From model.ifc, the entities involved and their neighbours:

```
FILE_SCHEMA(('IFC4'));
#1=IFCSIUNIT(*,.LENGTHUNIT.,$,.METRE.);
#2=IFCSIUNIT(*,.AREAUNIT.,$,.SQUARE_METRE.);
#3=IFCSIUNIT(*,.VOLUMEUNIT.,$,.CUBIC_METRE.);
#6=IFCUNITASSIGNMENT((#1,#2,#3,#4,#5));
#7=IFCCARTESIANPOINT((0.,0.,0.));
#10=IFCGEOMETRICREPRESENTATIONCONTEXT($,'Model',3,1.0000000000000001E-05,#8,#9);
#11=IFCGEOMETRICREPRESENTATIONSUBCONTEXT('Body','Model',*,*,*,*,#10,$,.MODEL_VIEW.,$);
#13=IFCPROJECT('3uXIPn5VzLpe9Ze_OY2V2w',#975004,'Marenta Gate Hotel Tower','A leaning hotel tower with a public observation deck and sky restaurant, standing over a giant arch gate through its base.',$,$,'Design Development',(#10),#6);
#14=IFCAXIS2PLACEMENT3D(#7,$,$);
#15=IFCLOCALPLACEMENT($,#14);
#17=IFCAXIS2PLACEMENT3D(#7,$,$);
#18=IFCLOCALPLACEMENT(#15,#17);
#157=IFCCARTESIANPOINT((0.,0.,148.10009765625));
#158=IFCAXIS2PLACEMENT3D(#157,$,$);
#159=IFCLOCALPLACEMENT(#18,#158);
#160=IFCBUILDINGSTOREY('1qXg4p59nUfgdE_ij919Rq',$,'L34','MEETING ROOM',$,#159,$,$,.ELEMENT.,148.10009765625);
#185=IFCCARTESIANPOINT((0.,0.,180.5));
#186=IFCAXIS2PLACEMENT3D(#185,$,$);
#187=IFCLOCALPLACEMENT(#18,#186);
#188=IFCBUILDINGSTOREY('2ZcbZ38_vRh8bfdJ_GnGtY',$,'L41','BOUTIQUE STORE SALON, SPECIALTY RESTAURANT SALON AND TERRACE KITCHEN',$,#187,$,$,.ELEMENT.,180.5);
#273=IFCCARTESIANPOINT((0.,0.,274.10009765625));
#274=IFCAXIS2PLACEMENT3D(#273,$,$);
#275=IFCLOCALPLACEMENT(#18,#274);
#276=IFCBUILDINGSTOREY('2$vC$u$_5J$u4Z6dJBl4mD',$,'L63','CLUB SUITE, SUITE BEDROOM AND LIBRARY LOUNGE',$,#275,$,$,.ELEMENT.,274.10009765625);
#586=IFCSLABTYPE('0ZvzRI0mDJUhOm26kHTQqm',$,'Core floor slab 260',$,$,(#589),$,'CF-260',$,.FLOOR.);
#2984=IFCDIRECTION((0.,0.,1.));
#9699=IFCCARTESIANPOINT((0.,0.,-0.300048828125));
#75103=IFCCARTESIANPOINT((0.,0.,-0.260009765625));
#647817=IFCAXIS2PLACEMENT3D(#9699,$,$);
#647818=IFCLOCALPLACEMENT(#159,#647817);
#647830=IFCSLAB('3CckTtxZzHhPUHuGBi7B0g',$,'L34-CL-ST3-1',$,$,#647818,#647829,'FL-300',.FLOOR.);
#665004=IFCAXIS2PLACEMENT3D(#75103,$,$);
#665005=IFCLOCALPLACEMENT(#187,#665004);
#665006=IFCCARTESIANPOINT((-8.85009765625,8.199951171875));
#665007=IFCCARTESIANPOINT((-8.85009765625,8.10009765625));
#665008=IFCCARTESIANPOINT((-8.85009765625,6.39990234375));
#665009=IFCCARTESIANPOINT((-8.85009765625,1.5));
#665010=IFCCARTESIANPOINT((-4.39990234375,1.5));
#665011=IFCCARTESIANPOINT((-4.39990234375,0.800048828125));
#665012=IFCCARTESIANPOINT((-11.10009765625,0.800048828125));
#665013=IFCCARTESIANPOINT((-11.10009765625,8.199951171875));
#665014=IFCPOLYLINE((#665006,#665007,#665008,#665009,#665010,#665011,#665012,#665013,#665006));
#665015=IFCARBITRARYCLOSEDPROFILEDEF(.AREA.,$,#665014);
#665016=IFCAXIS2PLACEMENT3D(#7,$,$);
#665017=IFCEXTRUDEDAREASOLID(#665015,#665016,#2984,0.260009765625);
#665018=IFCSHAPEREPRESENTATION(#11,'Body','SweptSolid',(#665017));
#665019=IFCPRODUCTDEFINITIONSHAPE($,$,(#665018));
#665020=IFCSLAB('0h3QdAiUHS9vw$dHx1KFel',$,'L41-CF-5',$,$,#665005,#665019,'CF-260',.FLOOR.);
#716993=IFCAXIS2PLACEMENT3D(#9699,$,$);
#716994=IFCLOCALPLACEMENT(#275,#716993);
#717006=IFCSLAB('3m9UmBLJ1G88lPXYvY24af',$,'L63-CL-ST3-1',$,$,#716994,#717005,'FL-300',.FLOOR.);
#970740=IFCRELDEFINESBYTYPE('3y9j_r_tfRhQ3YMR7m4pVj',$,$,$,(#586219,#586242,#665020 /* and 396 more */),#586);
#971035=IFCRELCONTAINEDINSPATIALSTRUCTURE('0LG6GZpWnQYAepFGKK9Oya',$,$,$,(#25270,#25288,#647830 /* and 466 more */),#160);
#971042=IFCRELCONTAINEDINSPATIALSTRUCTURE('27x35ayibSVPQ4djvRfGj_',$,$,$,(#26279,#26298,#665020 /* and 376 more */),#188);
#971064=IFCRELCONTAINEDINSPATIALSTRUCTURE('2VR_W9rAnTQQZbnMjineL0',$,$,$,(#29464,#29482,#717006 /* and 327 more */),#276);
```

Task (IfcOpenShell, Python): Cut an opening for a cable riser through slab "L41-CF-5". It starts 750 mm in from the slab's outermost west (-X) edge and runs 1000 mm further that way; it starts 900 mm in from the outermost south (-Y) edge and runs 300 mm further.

```python
import numpy as np
import ifcopenshell
import ifcopenshell.api.feature
import ifcopenshell.api.geometry
import ifcopenshell.api.root
import ifcopenshell.geom
import ifcopenshell.util.placement
import ifcopenshell.util.representation
import ifcopenshell.util.shape
import ifcopenshell.util.unit

model = ifcopenshell.open("model.ifc")
unit_scale = ifcopenshell.util.unit.calculate_unit_scale(model)
settings = ifcopenshell.geom.settings()


def volume(element):
    """Net volume in cubic metres, openings subtracted."""
    shape = ifcopenshell.geom.create_shape(settings, element)
    return ifcopenshell.util.shape.get_volume(shape.geometry)


slab = model.by_guid("0h3QdAiUHS9vw$dHx1KFel")
before = volume(slab)

# Extent in the slab's own axes, in metres. The edges named are its -X and -Y sides.
slab_shape = ifcopenshell.geom.create_shape(settings, slab)
vertices = ifcopenshell.util.shape.get_vertices(slab_shape.geometry)
x_min, y_min, bottom = vertices.min(axis=0)
top = vertices[:, 2].max()

opening = ifcopenshell.api.root.create_entity(model, ifc_class="IfcOpeningElement", name="Cable riser opening", predefined_type="OPENING")
context = ifcopenshell.util.representation.get_context(model, "Model", "Body", "MODEL_VIEW")
width, depth = 1, 0.3
outline = [(0.0, 0.0), (width, 0.0), (width, depth), (0.0, depth), (0.0, 0.0)]
# Overshoot both faces by 50 mm so the cut is clean.
shape = ifcopenshell.api.geometry.add_slab_representation(
    model, context=context, depth=top - bottom + 0.1, polyline=outline
)
ifcopenshell.api.geometry.assign_representation(model, product=opening, representation=shape)

matrix = ifcopenshell.util.placement.get_local_placement(slab.ObjectPlacement)
matrix[:, 3] = matrix @ np.append(np.array([x_min + 0.75, y_min + 0.9, bottom - 0.05]) / unit_scale, 1.0)
ifcopenshell.api.geometry.edit_object_placement(model, product=opening, matrix=matrix, is_si=False)
ifcopenshell.api.feature.add_feature(model, feature=opening, element=slab)

after = volume(slab)

print(f"slab volume {before:.3f} -> {after:.3f} m3")

model.write("model_updated.ifc")
```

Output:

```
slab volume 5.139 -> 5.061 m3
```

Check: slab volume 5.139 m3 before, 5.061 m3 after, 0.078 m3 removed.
